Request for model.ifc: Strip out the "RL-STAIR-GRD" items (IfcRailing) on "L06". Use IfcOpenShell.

First a look at what the model holds.

```python
import ifcopenshell
import ifcopenshell.util.element

model = ifcopenshell.open("model.ifc")
print(model.schema)
storey = next(s for s in model.by_type("IfcBuildingStorey") if s.Name == "L06")
railings = [e for e in ifcopenshell.util.element.get_decomposition(storey) if e.is_a("IfcRailing")]
seen = {}
for e in railings:
    element_type = ifcopenshell.util.element.get_type(e)
    name = element_type.Name if element_type not in (None, e) else None
    seen[name] = seen.get(name, 0) + 1
for name, count in sorted(seen.items(), key=str):
    print(count, "x", name)
```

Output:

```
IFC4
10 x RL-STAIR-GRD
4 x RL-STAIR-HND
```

```python
import ifcopenshell
import ifcopenshell.api.root
import ifcopenshell.util.element

model = ifcopenshell.open("model.ifc")

storey = next(s for s in model.by_type("IfcBuildingStorey") if s.Name == "L06")
railings = [e for e in ifcopenshell.util.element.get_decomposition(storey) if e.is_a("IfcRailing")]
targets = [e for e in railings if (t := ifcopenshell.util.element.get_type(e)) not in (None, e) and t.Name == "RL-STAIR-GRD"]

for e in targets:
    ifcopenshell.api.root.remove_product(model, product=e)
print(len(targets), "removed")

model.write("model_edited.ifc")
```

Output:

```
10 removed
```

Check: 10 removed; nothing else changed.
